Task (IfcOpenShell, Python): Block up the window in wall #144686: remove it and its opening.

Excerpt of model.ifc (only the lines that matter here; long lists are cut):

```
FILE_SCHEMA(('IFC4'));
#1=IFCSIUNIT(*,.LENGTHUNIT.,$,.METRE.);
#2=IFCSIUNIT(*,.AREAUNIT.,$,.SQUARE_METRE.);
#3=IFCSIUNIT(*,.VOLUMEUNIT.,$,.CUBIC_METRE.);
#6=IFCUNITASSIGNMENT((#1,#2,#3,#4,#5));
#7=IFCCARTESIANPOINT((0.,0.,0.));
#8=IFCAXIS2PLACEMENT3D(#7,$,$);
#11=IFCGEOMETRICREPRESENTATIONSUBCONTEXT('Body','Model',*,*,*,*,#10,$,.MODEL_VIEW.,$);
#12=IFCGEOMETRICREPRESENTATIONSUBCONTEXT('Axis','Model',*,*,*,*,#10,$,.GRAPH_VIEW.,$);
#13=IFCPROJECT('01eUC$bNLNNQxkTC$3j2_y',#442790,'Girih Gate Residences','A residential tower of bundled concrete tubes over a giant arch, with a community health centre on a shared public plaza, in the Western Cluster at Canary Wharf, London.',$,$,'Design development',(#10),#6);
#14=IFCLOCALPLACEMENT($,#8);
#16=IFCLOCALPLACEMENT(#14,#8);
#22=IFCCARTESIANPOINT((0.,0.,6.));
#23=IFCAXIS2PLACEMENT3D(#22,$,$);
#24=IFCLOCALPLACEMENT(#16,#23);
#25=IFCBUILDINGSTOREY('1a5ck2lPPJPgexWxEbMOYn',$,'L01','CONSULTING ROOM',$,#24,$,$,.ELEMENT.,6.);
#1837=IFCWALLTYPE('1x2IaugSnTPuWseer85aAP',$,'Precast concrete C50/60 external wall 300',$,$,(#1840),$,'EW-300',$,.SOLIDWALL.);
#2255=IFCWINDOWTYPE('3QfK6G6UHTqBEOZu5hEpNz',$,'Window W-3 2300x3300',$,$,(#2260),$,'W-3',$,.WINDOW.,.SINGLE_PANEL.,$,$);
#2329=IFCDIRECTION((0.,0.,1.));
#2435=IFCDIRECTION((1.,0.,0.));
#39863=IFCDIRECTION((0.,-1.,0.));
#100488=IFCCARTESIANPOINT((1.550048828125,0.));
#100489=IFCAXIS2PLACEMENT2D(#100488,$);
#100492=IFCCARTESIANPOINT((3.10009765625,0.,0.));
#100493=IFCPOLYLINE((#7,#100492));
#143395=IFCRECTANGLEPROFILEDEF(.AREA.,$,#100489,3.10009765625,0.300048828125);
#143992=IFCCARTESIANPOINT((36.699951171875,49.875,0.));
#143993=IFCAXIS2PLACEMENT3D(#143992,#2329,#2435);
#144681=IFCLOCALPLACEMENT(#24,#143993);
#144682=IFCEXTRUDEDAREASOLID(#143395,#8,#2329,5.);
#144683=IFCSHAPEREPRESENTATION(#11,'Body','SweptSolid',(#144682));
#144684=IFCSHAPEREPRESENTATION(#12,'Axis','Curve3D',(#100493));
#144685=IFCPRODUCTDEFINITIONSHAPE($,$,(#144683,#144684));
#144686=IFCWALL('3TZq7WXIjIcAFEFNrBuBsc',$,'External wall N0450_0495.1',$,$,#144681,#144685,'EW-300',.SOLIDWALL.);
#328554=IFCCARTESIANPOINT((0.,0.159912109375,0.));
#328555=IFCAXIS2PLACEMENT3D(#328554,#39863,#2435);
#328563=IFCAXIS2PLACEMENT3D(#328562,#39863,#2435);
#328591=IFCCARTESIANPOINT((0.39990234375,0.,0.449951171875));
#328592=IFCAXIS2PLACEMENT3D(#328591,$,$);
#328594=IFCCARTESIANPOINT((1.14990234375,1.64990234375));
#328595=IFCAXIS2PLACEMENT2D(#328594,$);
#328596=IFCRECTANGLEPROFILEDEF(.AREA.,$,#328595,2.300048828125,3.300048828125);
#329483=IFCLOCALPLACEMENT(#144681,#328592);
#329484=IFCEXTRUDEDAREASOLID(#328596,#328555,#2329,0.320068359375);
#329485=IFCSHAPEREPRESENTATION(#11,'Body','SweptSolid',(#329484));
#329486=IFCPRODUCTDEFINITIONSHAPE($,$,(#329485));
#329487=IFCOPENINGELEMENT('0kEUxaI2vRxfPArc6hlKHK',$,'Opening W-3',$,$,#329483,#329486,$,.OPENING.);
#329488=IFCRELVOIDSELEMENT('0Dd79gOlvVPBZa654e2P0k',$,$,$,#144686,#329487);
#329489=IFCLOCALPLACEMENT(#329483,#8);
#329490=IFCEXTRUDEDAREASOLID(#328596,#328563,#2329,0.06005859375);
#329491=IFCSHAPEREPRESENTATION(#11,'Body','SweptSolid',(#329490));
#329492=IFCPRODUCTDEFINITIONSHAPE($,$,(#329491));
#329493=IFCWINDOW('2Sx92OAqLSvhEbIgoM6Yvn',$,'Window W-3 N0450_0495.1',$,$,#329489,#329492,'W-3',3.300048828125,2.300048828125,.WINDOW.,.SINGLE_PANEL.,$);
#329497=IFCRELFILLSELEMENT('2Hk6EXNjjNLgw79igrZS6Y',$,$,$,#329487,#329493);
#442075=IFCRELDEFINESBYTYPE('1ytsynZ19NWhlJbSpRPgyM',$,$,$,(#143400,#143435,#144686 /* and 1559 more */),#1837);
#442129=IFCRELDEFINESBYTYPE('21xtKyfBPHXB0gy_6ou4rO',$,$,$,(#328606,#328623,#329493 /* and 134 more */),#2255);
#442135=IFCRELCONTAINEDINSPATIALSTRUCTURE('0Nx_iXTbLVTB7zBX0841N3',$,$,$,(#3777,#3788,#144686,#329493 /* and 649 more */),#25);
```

```python
import ifcopenshell
import ifcopenshell.api.feature
import ifcopenshell.api.root
import ifcopenshell.geom
import ifcopenshell.util.shape

model = ifcopenshell.open("model.ifc")
settings = ifcopenshell.geom.settings()


def volume(element):
    """Net volume in cubic metres, openings subtracted."""
    shape = ifcopenshell.geom.create_shape(settings, element)
    return ifcopenshell.util.shape.get_volume(shape.geometry)


window = model.by_guid("2Sx92OAqLSvhEbIgoM6Yvn")
opening = window.FillsVoids[0].RelatingOpeningElement
wall = opening.VoidsElements[0].RelatingBuildingElement
before = volume(wall)

ifcopenshell.api.root.remove_product(model, product=window)
ifcopenshell.api.feature.remove_feature(model, feature=opening)

after = volume(wall)

print(f"wall volume {before:.3f} -> {after:.3f} m3")

model.write("model_v2.ifc")
```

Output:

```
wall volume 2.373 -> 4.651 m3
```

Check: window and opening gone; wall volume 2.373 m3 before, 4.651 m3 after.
